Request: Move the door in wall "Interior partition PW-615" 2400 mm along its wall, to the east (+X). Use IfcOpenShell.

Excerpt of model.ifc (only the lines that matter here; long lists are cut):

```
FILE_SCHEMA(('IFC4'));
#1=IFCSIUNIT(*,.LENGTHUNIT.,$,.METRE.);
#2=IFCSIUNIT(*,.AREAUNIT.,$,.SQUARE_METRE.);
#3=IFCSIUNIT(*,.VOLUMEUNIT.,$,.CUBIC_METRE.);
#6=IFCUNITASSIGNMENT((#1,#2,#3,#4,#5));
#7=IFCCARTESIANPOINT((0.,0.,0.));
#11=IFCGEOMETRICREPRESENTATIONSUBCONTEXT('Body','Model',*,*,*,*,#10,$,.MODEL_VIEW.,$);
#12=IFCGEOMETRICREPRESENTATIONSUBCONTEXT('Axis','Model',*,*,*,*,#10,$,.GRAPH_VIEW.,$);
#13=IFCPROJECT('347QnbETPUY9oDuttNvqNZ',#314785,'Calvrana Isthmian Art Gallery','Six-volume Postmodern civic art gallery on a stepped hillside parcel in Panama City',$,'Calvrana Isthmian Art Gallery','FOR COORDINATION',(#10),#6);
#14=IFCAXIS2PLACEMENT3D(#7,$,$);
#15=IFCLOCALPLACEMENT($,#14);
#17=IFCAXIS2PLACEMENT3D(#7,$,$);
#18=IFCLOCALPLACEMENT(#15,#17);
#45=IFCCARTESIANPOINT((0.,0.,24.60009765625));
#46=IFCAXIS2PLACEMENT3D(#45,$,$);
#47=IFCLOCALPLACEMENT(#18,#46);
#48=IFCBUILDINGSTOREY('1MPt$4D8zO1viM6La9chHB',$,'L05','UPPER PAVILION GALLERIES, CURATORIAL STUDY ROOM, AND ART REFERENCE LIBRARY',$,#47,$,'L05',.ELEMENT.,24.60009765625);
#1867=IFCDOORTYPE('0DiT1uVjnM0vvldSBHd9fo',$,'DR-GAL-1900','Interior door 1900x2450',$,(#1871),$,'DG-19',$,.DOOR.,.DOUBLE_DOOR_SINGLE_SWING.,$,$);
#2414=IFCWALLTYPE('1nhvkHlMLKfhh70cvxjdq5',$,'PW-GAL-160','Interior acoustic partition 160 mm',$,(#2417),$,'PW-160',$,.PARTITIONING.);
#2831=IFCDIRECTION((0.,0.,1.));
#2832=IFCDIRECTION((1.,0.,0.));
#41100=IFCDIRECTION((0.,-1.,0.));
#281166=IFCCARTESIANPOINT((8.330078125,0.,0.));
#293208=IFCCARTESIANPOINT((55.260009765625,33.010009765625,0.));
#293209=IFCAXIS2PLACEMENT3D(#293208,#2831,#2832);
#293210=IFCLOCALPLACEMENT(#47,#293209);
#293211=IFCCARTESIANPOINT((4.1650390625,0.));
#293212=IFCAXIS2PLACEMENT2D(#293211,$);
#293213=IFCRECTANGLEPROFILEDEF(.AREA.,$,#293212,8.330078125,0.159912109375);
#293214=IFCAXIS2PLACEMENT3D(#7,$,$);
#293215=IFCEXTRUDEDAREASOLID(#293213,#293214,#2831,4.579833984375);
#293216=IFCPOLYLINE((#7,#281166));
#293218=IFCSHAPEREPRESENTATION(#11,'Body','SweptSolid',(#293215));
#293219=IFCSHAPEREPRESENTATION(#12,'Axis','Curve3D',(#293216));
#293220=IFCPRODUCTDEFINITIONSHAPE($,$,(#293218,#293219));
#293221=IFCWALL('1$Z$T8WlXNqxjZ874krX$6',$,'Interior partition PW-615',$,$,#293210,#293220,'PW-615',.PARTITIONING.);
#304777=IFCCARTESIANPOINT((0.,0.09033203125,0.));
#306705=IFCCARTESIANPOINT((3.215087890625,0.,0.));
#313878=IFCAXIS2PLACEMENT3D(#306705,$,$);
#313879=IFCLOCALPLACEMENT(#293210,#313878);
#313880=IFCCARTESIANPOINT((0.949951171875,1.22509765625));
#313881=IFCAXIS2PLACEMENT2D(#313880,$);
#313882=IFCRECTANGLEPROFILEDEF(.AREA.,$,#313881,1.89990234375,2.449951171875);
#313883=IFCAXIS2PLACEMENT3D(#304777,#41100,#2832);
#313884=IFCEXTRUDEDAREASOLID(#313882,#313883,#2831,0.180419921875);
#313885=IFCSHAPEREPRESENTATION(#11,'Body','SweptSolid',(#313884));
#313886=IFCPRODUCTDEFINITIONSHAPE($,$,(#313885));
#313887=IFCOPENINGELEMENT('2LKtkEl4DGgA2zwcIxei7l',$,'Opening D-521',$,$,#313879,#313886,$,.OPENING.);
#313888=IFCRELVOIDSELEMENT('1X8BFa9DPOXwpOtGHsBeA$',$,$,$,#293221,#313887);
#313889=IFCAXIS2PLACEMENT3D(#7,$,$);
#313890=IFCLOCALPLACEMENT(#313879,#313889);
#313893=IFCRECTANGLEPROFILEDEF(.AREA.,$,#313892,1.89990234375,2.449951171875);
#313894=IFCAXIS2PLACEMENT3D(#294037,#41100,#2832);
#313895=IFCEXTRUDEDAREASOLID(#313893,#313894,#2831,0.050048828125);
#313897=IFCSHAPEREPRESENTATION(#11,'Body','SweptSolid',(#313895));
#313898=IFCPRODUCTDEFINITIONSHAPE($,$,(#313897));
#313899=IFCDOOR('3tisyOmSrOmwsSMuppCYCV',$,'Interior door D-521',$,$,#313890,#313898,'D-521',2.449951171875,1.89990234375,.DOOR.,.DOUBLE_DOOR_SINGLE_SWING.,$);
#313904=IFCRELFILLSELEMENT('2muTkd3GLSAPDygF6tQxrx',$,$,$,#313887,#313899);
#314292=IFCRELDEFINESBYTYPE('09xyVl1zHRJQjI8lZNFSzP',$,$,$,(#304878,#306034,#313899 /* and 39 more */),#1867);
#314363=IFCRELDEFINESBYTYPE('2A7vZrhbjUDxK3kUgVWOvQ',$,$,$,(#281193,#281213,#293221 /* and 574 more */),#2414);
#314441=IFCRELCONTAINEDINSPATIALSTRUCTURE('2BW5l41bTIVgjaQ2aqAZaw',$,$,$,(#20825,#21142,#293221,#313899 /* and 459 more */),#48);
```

```python
import ifcopenshell
import ifcopenshell.api.geometry
import ifcopenshell.util.placement
import ifcopenshell.util.unit

model = ifcopenshell.open("model.ifc")
unit_scale = ifcopenshell.util.unit.calculate_unit_scale(model)

door = model.by_guid("3tisyOmSrOmwsSMuppCYCV")
opening = door.FillsVoids[0].RelatingOpeningElement
wall = opening.VoidsElements[0].RelatingBuildingElement

wall_matrix = ifcopenshell.util.placement.get_local_placement(wall.ObjectPlacement)
shift = wall_matrix[:3, 0] * 2.4 / unit_scale
before = ifcopenshell.util.placement.get_local_placement(door.ObjectPlacement)[:3, 3].copy()

# The door is placed relative to its opening, so it follows when the opening moves.
matrix = ifcopenshell.util.placement.get_local_placement(opening.ObjectPlacement)
matrix[:3, 3] += shift
ifcopenshell.api.geometry.edit_object_placement(
    model, product=opening, matrix=matrix, is_si=False, should_transform_children=True
)

after = ifcopenshell.util.placement.get_local_placement(door.ObjectPlacement)[:3, 3]
print("door moved by", (after - before).round(3) + 0.0)

model.write("model_updated.ifc")
```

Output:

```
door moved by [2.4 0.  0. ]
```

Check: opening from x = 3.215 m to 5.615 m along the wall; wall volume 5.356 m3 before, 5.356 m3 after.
